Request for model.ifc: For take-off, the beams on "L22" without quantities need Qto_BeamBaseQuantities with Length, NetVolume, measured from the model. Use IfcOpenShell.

First a look at what the model holds.

```python
import ifcopenshell
import ifcopenshell.util.element
import ifcopenshell.util.unit

model = ifcopenshell.open("model.ifc")
print(model.schema)
for unit_type in ("LENGTHUNIT", "AREAUNIT", "VOLUMEUNIT"):
    print(unit_type, ifcopenshell.util.unit.calculate_unit_scale(model, unit_type))
storey = next(s for s in model.by_type("IfcBuildingStorey") if s.Name == "L22")
beams = [e for e in ifcopenshell.util.element.get_decomposition(storey) if e.is_a("IfcBeam")]
for e in sorted(beams, key=lambda e: e.id()):
    print(e.id(), e.is_a(), e.Name, list(ifcopenshell.util.element.get_psets(e, qtos_only=True)), sep=" | ")
```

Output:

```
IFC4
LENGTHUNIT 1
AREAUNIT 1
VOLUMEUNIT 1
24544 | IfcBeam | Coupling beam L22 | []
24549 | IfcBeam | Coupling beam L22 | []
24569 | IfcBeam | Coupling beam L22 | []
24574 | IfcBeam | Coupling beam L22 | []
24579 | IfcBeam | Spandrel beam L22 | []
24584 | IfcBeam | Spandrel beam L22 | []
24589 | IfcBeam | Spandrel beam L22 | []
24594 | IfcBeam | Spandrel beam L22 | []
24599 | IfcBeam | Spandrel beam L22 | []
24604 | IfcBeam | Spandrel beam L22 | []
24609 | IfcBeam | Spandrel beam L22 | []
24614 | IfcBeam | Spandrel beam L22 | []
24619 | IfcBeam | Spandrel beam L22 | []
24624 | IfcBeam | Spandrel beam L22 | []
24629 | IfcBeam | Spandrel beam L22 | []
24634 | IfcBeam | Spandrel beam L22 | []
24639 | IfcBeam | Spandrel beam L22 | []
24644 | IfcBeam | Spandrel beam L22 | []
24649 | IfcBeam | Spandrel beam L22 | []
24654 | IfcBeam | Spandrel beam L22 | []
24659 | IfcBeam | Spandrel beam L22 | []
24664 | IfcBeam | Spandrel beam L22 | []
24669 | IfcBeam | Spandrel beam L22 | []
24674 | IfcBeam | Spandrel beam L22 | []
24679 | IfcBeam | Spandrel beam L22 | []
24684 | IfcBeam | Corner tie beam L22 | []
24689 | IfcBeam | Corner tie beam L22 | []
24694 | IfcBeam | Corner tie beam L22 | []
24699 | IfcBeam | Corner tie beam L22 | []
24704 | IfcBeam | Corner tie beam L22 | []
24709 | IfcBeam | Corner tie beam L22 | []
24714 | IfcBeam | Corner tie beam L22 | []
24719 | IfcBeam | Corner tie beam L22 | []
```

```python
import ifcopenshell
import ifcopenshell.api.pset
import ifcopenshell.geom
import ifcopenshell.util.element
import ifcopenshell.util.shape
import ifcopenshell.util.unit

model = ifcopenshell.open("model.ifc")
unit_scale = ifcopenshell.util.unit.calculate_unit_scale(model)
volume_scale = ifcopenshell.util.unit.calculate_unit_scale(model, "VOLUMEUNIT")
settings = ifcopenshell.geom.settings()

storey = next(s for s in model.by_type("IfcBuildingStorey") if s.Name == "L22")
beams = [e for e in ifcopenshell.util.element.get_decomposition(storey) if e.is_a("IfcBeam")]

for e in sorted(beams, key=lambda e: e.id()):
    if ifcopenshell.util.element.get_psets(e, qtos_only=True, should_inherit=False):
        continue
    # Geometry comes back in metres, in the element's own axes.
    shape = ifcopenshell.geom.create_shape(settings, e)
    values = {
        "Length": ifcopenshell.util.shape.get_max_xyz(shape.geometry) / unit_scale,
        "NetVolume": ifcopenshell.util.shape.get_volume(shape.geometry) / volume_scale,
    }
    qto = ifcopenshell.api.pset.add_qto(model, product=e, name="Qto_BeamBaseQuantities")
    ifcopenshell.api.pset.edit_qto(model, qto=qto, properties=values)
    print(e.id(), {k: round(v, 3) for k, v in values.items()})

model.write("model_updated.ifc")
```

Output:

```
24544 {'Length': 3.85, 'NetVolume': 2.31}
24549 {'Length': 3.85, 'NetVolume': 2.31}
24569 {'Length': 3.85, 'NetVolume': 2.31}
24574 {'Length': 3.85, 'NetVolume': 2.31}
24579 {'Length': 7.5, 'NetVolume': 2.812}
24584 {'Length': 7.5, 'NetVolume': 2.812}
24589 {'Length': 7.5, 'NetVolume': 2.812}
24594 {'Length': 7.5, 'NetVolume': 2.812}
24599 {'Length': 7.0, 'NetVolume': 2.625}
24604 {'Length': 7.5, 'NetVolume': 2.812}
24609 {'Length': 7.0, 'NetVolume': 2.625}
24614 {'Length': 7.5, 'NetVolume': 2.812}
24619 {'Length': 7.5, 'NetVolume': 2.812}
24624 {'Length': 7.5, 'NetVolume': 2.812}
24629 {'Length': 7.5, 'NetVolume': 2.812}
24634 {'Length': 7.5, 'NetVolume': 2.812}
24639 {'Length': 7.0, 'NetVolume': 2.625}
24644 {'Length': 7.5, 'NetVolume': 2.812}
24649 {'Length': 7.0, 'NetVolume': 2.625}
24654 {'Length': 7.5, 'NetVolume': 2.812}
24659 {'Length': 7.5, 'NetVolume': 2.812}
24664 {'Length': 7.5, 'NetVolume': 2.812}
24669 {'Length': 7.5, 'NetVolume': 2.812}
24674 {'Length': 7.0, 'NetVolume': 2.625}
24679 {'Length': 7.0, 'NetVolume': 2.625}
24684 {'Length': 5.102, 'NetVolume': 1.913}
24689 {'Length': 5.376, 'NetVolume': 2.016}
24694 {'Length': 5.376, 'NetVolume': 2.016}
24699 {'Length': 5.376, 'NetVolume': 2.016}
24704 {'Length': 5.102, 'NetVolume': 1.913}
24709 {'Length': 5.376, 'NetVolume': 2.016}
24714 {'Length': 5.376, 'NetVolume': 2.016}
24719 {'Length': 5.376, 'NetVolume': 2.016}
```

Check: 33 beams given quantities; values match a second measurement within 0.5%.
